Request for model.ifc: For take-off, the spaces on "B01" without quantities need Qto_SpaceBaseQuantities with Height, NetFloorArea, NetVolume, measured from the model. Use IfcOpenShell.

First a look at what the model holds.

```python
import ifcopenshell
import ifcopenshell.util.element
import ifcopenshell.util.unit

model = ifcopenshell.open("model.ifc")
print(model.schema)
for unit_type in ("LENGTHUNIT", "AREAUNIT", "VOLUMEUNIT"):
    print(unit_type, ifcopenshell.util.unit.calculate_unit_scale(model, unit_type))
storey = next(s for s in model.by_type("IfcBuildingStorey") if s.Name == "B01")
spaces = [e for e in ifcopenshell.util.element.get_decomposition(storey) if e.is_a("IfcSpace")]
for e in sorted(spaces, key=lambda e: e.id()):
    print(e.id(), e.is_a(), e.Name, list(ifcopenshell.util.element.get_psets(e, qtos_only=True)), sep=" | ")
```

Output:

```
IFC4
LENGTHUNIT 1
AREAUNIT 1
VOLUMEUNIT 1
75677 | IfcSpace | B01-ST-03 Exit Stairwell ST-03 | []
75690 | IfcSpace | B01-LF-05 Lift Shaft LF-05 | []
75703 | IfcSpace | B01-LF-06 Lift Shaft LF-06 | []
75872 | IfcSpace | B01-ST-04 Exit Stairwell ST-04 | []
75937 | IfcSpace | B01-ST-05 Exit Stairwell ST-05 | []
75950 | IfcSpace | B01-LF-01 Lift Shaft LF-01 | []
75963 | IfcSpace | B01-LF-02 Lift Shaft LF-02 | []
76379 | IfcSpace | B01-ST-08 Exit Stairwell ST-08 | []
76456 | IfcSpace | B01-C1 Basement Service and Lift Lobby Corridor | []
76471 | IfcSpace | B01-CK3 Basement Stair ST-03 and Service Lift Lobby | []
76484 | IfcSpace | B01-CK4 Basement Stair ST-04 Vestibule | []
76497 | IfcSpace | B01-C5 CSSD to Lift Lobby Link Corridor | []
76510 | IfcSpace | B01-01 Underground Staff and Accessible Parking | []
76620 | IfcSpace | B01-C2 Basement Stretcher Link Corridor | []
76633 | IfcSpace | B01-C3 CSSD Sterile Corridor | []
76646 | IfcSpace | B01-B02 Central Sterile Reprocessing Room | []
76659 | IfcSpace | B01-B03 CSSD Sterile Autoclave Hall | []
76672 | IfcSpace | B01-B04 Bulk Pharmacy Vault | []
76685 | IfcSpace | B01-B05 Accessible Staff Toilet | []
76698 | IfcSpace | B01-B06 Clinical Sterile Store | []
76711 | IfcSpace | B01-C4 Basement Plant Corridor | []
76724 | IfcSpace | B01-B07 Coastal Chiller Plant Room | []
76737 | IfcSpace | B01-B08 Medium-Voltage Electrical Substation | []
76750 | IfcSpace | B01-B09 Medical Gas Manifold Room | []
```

```python
import ifcopenshell
import ifcopenshell.api.pset
import ifcopenshell.geom
import ifcopenshell.util.element
import ifcopenshell.util.shape
import ifcopenshell.util.unit

model = ifcopenshell.open("model.ifc")
unit_scale = ifcopenshell.util.unit.calculate_unit_scale(model)
area_scale = ifcopenshell.util.unit.calculate_unit_scale(model, "AREAUNIT")
volume_scale = ifcopenshell.util.unit.calculate_unit_scale(model, "VOLUMEUNIT")
settings = ifcopenshell.geom.settings()

storey = next(s for s in model.by_type("IfcBuildingStorey") if s.Name == "B01")
spaces = [e for e in ifcopenshell.util.element.get_decomposition(storey) if e.is_a("IfcSpace")]

for e in sorted(spaces, key=lambda e: e.id()):
    if ifcopenshell.util.element.get_psets(e, qtos_only=True, should_inherit=False):
        continue
    # Geometry comes back in metres, in the element's own axes.
    shape = ifcopenshell.geom.create_shape(settings, e)
    values = {
        "Height": ifcopenshell.util.shape.get_z(shape.geometry) / unit_scale,
        "NetFloorArea": ifcopenshell.util.shape.get_footprint_area(shape.geometry) / area_scale,
        "NetVolume": ifcopenshell.util.shape.get_volume(shape.geometry) / volume_scale,
    }
    qto = ifcopenshell.api.pset.add_qto(model, product=e, name="Qto_SpaceBaseQuantities")
    ifcopenshell.api.pset.edit_qto(model, qto=qto, properties=values)
    print(e.id(), {k: round(v, 3) for k, v in values.items()})

model.write("model_edited.ifc")
```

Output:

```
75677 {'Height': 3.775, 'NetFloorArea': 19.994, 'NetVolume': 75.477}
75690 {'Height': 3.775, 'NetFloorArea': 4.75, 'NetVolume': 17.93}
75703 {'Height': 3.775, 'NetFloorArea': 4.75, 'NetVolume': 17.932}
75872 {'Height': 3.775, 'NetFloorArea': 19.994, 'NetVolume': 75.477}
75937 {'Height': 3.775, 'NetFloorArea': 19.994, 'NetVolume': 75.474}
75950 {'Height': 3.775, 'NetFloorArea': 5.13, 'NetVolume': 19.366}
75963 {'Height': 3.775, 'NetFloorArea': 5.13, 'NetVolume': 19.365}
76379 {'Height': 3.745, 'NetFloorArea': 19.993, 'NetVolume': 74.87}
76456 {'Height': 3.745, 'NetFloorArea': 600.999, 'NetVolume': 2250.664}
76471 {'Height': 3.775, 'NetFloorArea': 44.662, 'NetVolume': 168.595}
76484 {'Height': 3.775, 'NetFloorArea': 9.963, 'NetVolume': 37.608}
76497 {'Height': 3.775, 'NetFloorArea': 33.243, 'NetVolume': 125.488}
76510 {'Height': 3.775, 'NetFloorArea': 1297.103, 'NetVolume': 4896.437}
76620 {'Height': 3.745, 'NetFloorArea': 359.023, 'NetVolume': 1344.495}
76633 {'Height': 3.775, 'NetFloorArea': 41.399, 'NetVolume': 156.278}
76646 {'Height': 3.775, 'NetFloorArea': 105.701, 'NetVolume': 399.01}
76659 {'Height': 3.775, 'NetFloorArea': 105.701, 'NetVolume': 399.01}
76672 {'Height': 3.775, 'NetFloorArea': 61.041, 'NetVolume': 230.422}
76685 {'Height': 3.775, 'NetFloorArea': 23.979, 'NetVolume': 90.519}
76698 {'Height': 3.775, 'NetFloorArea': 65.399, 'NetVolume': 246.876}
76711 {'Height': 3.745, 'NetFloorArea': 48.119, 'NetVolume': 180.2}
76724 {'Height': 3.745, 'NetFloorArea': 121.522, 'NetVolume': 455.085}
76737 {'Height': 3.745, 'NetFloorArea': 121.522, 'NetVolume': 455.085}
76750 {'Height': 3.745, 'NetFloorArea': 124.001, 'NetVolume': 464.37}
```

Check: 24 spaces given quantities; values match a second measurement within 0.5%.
